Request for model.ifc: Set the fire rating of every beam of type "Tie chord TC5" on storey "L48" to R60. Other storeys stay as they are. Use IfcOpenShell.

First a look at what the model holds.

```python
import ifcopenshell
import ifcopenshell.util.element

model = ifcopenshell.open("model.ifc")
print(model.schema)
storey = next(s for s in model.by_type("IfcBuildingStorey") if s.Name == "L48")
beams = [e for e in ifcopenshell.util.element.get_decomposition(storey) if e.is_a("IfcBeam")]
seen = {}
for e in beams:
    element_type = ifcopenshell.util.element.get_type(e)
    key = (element_type.Name if element_type != e and element_type else None, ifcopenshell.util.element.get_pset(e, "Pset_BeamCommon", "FireRating"))
    seen[key] = seen.get(key, 0) + 1
for (name, value), count in sorted(seen.items(), key=str):
    print(count, "x", name, "|", value)
```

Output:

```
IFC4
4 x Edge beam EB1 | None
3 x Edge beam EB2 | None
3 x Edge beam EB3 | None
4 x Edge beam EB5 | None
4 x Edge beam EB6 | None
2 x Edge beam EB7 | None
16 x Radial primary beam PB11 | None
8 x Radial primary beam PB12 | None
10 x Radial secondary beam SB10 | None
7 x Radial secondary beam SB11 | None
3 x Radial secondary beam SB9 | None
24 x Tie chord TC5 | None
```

```python
import ifcopenshell
import ifcopenshell.api.pset
import ifcopenshell.util.element

model = ifcopenshell.open("model.ifc")

storey = next(s for s in model.by_type("IfcBuildingStorey") if s.Name == "L48")
beams = [e for e in ifcopenshell.util.element.get_decomposition(storey) if e.is_a("IfcBeam")]

count = 0
for e in beams:
    element_type = ifcopenshell.util.element.get_type(e)
    if element_type in (None, e) or element_type.Name != "Tie chord TC5":
        continue
    found = ifcopenshell.util.element.get_pset(e, "Pset_BeamCommon", should_inherit=False)
    if found:
        pset = model.by_id(found["id"])
        if len(ifcopenshell.util.element.get_elements_by_pset(pset)) > 1:
            pset = ifcopenshell.api.pset.unshare_pset(model, products=[e], pset=pset)[0]
    else:
        pset = ifcopenshell.api.pset.add_pset(model, product=e, name="Pset_BeamCommon")
    ifcopenshell.api.pset.edit_pset(model, pset=pset, properties={"FireRating": "R60"})
    count += 1

print(count, "beams updated")

model.write("model_v2.ifc")
```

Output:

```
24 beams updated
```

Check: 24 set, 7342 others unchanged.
